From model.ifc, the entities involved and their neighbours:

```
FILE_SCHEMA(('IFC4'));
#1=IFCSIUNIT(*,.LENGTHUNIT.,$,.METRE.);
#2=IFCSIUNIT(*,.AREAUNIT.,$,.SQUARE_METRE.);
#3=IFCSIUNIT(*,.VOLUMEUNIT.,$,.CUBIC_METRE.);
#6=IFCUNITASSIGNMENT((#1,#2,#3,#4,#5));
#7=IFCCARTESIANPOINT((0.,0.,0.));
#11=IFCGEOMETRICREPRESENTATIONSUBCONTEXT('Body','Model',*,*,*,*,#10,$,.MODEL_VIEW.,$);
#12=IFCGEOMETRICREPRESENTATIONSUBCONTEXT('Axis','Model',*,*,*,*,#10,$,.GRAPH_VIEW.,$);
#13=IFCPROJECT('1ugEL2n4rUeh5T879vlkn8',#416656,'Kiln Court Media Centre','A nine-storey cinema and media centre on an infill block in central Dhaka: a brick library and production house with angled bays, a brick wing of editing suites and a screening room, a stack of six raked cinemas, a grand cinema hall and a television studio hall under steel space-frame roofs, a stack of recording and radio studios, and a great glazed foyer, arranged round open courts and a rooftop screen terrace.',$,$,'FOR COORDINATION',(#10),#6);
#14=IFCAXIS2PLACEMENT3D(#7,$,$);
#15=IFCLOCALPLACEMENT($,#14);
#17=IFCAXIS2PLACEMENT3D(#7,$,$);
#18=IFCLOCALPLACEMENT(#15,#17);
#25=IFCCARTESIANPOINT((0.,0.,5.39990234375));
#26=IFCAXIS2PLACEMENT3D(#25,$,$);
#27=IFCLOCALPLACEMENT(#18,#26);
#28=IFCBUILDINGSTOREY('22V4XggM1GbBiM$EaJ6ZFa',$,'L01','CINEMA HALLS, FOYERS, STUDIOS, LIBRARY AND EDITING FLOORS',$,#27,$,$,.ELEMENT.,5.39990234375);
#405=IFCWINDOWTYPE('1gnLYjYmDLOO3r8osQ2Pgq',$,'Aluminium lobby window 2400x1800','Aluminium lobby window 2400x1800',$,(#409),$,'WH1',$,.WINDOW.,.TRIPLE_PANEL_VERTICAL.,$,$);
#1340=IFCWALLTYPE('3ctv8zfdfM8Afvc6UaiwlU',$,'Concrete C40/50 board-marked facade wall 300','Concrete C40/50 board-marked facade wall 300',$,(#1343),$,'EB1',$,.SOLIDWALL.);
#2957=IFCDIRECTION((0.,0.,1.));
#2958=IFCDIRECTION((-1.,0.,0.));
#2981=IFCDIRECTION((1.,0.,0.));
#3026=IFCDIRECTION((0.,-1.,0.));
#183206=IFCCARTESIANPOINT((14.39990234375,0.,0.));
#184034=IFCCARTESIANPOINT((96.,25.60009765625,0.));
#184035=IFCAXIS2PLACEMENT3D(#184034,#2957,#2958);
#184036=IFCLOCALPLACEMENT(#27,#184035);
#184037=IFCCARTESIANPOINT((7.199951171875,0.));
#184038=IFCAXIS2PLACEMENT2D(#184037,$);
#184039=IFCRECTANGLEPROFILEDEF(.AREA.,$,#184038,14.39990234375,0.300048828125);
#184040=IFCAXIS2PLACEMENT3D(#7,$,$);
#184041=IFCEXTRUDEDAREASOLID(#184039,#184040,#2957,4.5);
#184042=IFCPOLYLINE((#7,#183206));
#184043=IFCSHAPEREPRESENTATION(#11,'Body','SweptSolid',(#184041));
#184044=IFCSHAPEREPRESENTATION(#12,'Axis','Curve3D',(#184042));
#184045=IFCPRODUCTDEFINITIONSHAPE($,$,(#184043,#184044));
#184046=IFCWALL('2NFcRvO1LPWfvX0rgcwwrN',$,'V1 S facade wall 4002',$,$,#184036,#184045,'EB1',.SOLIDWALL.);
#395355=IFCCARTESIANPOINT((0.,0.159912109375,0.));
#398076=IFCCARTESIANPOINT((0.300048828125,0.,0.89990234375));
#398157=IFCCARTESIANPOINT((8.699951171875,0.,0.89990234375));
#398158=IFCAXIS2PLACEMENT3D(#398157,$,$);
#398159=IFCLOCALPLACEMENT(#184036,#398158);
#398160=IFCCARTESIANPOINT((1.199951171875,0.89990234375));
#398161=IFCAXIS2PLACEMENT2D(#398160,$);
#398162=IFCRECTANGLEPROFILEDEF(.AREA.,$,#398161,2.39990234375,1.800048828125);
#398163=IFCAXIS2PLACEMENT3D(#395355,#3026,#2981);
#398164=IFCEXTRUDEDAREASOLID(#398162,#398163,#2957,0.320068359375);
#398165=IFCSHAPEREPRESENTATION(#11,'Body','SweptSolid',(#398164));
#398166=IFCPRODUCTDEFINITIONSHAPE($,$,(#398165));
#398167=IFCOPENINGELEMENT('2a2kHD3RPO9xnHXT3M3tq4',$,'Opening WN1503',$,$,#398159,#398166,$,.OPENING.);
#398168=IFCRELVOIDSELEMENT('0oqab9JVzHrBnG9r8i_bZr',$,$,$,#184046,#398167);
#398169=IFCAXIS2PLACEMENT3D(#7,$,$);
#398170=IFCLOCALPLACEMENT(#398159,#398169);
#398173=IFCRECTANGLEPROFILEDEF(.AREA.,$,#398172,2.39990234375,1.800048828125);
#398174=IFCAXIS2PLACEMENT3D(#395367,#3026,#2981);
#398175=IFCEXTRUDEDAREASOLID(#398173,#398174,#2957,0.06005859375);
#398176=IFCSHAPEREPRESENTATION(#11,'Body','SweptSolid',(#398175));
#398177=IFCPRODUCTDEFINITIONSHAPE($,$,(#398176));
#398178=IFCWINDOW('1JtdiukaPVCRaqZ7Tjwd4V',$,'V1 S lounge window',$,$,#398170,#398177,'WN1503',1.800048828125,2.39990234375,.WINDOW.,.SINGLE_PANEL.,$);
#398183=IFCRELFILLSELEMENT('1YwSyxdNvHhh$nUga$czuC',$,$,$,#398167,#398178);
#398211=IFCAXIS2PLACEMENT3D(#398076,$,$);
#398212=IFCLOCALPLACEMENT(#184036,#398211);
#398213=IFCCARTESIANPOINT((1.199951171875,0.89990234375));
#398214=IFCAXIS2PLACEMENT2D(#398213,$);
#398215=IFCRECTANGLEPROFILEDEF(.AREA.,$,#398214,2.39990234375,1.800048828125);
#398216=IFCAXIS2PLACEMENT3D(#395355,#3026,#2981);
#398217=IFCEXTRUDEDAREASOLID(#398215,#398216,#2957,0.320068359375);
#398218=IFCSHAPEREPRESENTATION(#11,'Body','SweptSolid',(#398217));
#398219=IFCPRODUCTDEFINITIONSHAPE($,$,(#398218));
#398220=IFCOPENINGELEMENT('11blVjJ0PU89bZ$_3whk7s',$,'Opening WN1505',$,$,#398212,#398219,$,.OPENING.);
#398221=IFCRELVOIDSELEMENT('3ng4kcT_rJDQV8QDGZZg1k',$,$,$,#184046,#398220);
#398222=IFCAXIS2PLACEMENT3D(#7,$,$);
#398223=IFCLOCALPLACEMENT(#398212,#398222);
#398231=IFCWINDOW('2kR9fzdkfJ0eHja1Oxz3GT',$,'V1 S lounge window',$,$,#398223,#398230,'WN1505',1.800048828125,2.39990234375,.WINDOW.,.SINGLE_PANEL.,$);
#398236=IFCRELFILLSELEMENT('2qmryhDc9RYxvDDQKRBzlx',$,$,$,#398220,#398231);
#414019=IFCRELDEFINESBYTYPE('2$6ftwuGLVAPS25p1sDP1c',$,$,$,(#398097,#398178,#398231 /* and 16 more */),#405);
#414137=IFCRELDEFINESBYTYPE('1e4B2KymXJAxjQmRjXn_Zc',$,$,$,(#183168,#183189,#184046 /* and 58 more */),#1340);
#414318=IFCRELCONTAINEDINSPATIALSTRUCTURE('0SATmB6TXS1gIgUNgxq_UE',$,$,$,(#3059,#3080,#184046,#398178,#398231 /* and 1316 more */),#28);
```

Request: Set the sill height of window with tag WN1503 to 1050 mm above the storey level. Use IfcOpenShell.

```python
import numpy as np
import ifcopenshell
import ifcopenshell.api.geometry
import ifcopenshell.geom
import ifcopenshell.util.element
import ifcopenshell.util.placement
import ifcopenshell.util.shape
import ifcopenshell.util.unit

model = ifcopenshell.open("model.ifc")
unit_scale = ifcopenshell.util.unit.calculate_unit_scale(model)

window = model.by_guid("1JtdiukaPVCRaqZ7Tjwd4V")
opening = window.FillsVoids[0].RelatingOpeningElement
storey = ifcopenshell.util.element.get_container(window, ifc_class="IfcBuildingStorey")
level = ifcopenshell.util.placement.get_local_placement(storey.ObjectPlacement)[2, 3]

# The opening's origin need not be at the sill, so measure its lowest point.
shape = ifcopenshell.geom.create_shape(ifcopenshell.geom.settings(), opening)
bottom = ifcopenshell.util.shape.get_shape_bottom_elevation(shape, shape.geometry) / unit_scale
dz = level + 1.05 - bottom

shift = np.array([0.0, 0.0, dz])
# The window is placed relative to its opening, so it follows when the opening moves.
matrix = ifcopenshell.util.placement.get_local_placement(opening.ObjectPlacement)
matrix[:3, 3] += shift
ifcopenshell.api.geometry.edit_object_placement(
    model, product=opening, matrix=matrix, is_si=False, should_transform_children=True
)

print(f"moved by {dz * unit_scale:+.3f} m")

model.write("model_rev.ifc")
```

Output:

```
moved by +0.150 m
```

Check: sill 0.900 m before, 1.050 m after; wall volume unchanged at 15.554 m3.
